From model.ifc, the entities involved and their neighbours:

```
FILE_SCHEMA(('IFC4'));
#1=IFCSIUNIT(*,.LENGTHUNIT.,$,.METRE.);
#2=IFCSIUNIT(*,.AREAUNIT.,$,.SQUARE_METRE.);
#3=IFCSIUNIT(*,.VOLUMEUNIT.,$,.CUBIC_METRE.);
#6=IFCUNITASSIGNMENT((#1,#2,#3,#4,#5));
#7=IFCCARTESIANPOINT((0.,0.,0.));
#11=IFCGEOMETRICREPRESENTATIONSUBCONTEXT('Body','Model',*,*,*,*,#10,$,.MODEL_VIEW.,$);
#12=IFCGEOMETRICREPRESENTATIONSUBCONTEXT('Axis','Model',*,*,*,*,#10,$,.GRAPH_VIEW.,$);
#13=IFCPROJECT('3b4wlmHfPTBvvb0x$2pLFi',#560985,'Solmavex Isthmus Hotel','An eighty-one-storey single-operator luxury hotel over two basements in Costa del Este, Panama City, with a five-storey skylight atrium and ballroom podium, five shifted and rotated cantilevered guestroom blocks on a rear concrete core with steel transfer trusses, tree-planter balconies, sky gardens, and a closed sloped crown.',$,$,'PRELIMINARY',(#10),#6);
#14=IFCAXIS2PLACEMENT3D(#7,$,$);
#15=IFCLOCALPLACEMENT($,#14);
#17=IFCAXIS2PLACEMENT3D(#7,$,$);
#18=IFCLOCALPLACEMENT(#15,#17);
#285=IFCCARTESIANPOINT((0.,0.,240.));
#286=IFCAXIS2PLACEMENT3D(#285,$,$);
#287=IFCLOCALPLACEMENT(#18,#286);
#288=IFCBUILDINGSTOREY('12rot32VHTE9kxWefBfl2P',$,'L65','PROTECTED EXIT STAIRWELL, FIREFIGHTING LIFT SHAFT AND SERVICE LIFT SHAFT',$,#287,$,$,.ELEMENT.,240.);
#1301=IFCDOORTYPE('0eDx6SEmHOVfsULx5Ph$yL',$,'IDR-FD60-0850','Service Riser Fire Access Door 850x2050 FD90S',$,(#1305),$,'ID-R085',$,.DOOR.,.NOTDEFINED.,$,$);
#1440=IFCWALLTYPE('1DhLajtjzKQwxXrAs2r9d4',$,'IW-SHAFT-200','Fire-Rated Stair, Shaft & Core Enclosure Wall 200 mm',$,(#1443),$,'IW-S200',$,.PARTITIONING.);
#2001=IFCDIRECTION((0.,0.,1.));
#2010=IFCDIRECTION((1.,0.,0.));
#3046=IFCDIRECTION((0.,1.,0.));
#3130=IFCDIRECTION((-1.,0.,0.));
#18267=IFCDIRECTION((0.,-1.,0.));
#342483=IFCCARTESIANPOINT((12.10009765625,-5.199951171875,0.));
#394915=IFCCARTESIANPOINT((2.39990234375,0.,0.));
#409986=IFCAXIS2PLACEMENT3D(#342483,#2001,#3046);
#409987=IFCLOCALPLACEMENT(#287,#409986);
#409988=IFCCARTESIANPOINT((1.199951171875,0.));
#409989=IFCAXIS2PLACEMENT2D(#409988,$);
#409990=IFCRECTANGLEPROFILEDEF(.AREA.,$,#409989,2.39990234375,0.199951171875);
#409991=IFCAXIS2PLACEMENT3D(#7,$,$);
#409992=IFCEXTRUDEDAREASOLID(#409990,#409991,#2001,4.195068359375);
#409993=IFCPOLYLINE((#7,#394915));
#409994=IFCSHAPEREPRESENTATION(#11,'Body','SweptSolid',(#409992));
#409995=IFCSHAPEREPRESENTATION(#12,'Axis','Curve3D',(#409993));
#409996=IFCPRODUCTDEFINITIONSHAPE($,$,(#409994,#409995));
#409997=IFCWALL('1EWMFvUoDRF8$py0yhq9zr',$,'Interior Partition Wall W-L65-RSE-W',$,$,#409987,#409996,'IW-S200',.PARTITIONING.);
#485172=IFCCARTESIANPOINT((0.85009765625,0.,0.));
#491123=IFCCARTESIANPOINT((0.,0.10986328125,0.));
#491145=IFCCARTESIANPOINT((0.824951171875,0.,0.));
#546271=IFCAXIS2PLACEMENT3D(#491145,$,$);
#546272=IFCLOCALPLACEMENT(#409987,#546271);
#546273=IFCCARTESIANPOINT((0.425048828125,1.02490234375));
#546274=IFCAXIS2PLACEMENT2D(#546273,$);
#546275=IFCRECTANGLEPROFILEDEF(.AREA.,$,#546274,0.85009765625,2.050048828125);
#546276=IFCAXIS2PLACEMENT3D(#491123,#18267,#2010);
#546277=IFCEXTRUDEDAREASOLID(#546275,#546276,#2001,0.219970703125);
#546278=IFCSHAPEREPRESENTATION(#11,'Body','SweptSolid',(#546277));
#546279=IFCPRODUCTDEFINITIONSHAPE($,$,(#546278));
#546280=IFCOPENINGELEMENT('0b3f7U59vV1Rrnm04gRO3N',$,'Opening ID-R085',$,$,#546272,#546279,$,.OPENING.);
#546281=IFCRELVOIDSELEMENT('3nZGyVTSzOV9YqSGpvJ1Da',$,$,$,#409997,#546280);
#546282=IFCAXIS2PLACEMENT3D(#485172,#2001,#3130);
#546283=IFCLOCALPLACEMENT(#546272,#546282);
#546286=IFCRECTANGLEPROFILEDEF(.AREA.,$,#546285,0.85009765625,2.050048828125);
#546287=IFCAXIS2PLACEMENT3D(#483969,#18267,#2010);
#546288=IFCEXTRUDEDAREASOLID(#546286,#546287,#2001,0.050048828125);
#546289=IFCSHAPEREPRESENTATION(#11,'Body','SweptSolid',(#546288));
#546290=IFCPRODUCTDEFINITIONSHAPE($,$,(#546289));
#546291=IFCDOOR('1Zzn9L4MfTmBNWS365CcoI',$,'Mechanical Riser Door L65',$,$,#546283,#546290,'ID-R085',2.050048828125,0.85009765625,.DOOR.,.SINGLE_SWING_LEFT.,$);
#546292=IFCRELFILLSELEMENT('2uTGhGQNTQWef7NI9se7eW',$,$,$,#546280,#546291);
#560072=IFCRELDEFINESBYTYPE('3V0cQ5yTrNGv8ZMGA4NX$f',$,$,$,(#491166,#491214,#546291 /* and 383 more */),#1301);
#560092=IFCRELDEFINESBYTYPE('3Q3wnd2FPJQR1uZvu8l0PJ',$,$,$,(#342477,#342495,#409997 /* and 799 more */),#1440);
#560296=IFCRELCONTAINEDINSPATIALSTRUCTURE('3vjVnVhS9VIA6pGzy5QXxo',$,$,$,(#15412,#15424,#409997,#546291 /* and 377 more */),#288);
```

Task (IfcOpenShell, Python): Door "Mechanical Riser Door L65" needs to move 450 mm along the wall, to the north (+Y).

```python
import ifcopenshell
import ifcopenshell.api.geometry
import ifcopenshell.util.placement

model = ifcopenshell.open("model.ifc")

door = model.by_guid("1Zzn9L4MfTmBNWS365CcoI")
opening = door.FillsVoids[0].RelatingOpeningElement
wall = opening.VoidsElements[0].RelatingBuildingElement

wall_matrix = ifcopenshell.util.placement.get_local_placement(wall.ObjectPlacement)
shift = wall_matrix[:3, 0] * 0.45
before = ifcopenshell.util.placement.get_local_placement(door.ObjectPlacement)[:3, 3].copy()

# The door is placed relative to its opening, so it follows when the opening moves.
matrix = ifcopenshell.util.placement.get_local_placement(opening.ObjectPlacement)
matrix[:3, 3] += shift
ifcopenshell.api.geometry.edit_object_placement(
    model, product=opening, matrix=matrix, is_si=False, should_transform_children=True
)

after = ifcopenshell.util.placement.get_local_placement(door.ObjectPlacement)[:3, 3]
print("door moved by", (after - before).round(3) + 0.0)

model.write("model_updated.ifc")
```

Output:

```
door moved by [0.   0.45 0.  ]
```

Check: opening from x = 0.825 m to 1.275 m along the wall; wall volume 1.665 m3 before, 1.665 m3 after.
